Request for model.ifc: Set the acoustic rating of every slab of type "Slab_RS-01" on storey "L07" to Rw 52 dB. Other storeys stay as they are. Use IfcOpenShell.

First a look at what the model holds.

```python
import ifcopenshell
import ifcopenshell.util.element

model = ifcopenshell.open("model.ifc")
print(model.schema)
storey = next(s for s in model.by_type("IfcBuildingStorey") if s.Name == "L07")
slabs = [e for e in ifcopenshell.util.element.get_decomposition(storey) if e.is_a("IfcSlab")]
seen = {}
for e in slabs:
    element_type = ifcopenshell.util.element.get_type(e)
    key = (element_type.Name if element_type != e and element_type else None, ifcopenshell.util.element.get_pset(e, "Pset_SlabCommon", "AcousticRating"))
    seen[key] = seen.get(key, 0) + 1
for (name, value), count in sorted(seen.items(), key=str):
    print(count, "x", name, "|", value)
```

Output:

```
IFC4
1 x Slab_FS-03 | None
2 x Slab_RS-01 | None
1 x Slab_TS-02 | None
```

```python
import ifcopenshell
import ifcopenshell.api.pset
import ifcopenshell.util.element

model = ifcopenshell.open("model.ifc")

storey = next(s for s in model.by_type("IfcBuildingStorey") if s.Name == "L07")
slabs = [e for e in ifcopenshell.util.element.get_decomposition(storey) if e.is_a("IfcSlab")]

count = 0
for e in slabs:
    element_type = ifcopenshell.util.element.get_type(e)
    if element_type in (None, e) or element_type.Name != "Slab_RS-01":
        continue
    # add_pset returns the element's existing set when there is one.
    pset = ifcopenshell.api.pset.add_pset(model, product=e, name="Pset_SlabCommon")
    ifcopenshell.api.pset.edit_pset(model, pset=pset, properties={"AcousticRating": "Rw 52 dB"})
    count += 1

print(count, "slabs updated")

model.write("model_edited.ifc")
```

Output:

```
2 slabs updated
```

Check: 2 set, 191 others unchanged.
